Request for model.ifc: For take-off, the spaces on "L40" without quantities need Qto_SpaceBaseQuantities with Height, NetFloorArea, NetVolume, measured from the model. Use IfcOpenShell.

First a look at what the model holds.

```python
import ifcopenshell
import ifcopenshell.util.element
import ifcopenshell.util.unit

model = ifcopenshell.open("model.ifc")
print(model.schema)
for unit_type in ("LENGTHUNIT", "AREAUNIT", "VOLUMEUNIT"):
    print(unit_type, ifcopenshell.util.unit.calculate_unit_scale(model, unit_type))
storey = next(s for s in model.by_type("IfcBuildingStorey") if s.Name == "L40")
spaces = [e for e in ifcopenshell.util.element.get_decomposition(storey) if e.is_a("IfcSpace")]
for e in sorted(spaces, key=lambda e: e.id()):
    print(e.id(), e.is_a(), e.Name, list(ifcopenshell.util.element.get_psets(e, qtos_only=True)), sep=" | ")
```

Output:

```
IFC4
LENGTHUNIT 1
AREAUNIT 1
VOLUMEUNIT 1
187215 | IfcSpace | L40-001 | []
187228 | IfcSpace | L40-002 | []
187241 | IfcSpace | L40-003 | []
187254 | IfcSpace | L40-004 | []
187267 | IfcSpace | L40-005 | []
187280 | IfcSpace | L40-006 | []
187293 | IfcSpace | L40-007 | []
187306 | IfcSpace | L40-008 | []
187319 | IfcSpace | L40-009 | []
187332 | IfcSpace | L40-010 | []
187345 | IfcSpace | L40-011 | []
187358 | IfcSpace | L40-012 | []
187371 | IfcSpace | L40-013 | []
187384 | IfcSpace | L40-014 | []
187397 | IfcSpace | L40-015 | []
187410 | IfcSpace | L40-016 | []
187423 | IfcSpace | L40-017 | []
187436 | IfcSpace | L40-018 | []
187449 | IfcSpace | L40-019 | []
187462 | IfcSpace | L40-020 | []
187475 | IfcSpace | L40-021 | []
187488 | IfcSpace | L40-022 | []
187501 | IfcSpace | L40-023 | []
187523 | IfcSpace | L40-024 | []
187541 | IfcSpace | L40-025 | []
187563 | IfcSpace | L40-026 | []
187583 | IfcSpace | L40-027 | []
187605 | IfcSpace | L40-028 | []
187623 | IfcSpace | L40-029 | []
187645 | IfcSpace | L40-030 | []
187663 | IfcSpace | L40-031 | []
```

```python
import ifcopenshell
import ifcopenshell.api.pset
import ifcopenshell.geom
import ifcopenshell.util.element
import ifcopenshell.util.shape
import ifcopenshell.util.unit

model = ifcopenshell.open("model.ifc")
unit_scale = ifcopenshell.util.unit.calculate_unit_scale(model)
area_scale = ifcopenshell.util.unit.calculate_unit_scale(model, "AREAUNIT")
volume_scale = ifcopenshell.util.unit.calculate_unit_scale(model, "VOLUMEUNIT")
settings = ifcopenshell.geom.settings()

storey = next(s for s in model.by_type("IfcBuildingStorey") if s.Name == "L40")
spaces = [e for e in ifcopenshell.util.element.get_decomposition(storey) if e.is_a("IfcSpace")]

for e in sorted(spaces, key=lambda e: e.id()):
    if ifcopenshell.util.element.get_psets(e, qtos_only=True, should_inherit=False):
        continue
    # Geometry comes back in metres, in the element's own axes.
    shape = ifcopenshell.geom.create_shape(settings, e)
    values = {
        "Height": ifcopenshell.util.shape.get_z(shape.geometry) / unit_scale,
        "NetFloorArea": ifcopenshell.util.shape.get_footprint_area(shape.geometry) / area_scale,
        "NetVolume": ifcopenshell.util.shape.get_volume(shape.geometry) / volume_scale,
    }
    qto = ifcopenshell.api.pset.add_qto(model, product=e, name="Qto_SpaceBaseQuantities")
    ifcopenshell.api.pset.edit_qto(model, qto=qto, properties=values)
    print(e.id(), {k: round(v, 3) for k, v in values.items()})

model.write("model_edited.ifc")
```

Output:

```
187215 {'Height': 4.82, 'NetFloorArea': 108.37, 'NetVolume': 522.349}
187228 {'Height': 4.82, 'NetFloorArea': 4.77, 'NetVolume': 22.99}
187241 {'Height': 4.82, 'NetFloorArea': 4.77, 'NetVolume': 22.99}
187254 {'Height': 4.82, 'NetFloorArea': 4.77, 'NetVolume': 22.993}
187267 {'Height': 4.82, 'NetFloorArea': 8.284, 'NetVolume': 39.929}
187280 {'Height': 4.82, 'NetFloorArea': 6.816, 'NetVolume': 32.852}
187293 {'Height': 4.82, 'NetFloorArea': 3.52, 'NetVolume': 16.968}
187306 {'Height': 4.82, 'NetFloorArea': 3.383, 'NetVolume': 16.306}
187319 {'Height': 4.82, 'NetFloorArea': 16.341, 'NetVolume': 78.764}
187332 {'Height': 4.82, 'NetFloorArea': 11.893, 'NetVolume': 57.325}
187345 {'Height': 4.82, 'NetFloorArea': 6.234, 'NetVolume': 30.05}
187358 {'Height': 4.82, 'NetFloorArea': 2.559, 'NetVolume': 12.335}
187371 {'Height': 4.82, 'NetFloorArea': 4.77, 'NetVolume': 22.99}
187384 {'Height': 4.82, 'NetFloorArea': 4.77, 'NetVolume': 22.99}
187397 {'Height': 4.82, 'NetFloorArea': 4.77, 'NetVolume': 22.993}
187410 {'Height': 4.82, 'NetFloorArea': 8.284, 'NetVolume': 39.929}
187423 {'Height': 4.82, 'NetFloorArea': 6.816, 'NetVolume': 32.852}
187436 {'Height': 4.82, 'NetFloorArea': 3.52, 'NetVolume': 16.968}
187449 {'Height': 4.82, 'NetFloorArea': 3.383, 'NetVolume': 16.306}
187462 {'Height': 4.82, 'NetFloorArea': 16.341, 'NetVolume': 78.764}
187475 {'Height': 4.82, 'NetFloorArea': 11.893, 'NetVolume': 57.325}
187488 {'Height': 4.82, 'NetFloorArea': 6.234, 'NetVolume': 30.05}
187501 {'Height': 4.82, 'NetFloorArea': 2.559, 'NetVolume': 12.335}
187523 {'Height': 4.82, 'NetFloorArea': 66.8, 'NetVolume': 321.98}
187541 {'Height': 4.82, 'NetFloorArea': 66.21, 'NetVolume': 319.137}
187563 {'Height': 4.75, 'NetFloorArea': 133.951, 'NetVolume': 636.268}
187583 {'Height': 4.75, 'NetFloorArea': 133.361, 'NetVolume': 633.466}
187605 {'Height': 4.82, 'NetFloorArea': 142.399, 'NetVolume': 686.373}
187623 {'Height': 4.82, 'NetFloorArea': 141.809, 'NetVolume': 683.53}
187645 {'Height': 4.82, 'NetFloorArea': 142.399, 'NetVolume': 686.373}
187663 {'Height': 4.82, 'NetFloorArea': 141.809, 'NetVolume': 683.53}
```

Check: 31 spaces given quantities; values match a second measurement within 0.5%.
